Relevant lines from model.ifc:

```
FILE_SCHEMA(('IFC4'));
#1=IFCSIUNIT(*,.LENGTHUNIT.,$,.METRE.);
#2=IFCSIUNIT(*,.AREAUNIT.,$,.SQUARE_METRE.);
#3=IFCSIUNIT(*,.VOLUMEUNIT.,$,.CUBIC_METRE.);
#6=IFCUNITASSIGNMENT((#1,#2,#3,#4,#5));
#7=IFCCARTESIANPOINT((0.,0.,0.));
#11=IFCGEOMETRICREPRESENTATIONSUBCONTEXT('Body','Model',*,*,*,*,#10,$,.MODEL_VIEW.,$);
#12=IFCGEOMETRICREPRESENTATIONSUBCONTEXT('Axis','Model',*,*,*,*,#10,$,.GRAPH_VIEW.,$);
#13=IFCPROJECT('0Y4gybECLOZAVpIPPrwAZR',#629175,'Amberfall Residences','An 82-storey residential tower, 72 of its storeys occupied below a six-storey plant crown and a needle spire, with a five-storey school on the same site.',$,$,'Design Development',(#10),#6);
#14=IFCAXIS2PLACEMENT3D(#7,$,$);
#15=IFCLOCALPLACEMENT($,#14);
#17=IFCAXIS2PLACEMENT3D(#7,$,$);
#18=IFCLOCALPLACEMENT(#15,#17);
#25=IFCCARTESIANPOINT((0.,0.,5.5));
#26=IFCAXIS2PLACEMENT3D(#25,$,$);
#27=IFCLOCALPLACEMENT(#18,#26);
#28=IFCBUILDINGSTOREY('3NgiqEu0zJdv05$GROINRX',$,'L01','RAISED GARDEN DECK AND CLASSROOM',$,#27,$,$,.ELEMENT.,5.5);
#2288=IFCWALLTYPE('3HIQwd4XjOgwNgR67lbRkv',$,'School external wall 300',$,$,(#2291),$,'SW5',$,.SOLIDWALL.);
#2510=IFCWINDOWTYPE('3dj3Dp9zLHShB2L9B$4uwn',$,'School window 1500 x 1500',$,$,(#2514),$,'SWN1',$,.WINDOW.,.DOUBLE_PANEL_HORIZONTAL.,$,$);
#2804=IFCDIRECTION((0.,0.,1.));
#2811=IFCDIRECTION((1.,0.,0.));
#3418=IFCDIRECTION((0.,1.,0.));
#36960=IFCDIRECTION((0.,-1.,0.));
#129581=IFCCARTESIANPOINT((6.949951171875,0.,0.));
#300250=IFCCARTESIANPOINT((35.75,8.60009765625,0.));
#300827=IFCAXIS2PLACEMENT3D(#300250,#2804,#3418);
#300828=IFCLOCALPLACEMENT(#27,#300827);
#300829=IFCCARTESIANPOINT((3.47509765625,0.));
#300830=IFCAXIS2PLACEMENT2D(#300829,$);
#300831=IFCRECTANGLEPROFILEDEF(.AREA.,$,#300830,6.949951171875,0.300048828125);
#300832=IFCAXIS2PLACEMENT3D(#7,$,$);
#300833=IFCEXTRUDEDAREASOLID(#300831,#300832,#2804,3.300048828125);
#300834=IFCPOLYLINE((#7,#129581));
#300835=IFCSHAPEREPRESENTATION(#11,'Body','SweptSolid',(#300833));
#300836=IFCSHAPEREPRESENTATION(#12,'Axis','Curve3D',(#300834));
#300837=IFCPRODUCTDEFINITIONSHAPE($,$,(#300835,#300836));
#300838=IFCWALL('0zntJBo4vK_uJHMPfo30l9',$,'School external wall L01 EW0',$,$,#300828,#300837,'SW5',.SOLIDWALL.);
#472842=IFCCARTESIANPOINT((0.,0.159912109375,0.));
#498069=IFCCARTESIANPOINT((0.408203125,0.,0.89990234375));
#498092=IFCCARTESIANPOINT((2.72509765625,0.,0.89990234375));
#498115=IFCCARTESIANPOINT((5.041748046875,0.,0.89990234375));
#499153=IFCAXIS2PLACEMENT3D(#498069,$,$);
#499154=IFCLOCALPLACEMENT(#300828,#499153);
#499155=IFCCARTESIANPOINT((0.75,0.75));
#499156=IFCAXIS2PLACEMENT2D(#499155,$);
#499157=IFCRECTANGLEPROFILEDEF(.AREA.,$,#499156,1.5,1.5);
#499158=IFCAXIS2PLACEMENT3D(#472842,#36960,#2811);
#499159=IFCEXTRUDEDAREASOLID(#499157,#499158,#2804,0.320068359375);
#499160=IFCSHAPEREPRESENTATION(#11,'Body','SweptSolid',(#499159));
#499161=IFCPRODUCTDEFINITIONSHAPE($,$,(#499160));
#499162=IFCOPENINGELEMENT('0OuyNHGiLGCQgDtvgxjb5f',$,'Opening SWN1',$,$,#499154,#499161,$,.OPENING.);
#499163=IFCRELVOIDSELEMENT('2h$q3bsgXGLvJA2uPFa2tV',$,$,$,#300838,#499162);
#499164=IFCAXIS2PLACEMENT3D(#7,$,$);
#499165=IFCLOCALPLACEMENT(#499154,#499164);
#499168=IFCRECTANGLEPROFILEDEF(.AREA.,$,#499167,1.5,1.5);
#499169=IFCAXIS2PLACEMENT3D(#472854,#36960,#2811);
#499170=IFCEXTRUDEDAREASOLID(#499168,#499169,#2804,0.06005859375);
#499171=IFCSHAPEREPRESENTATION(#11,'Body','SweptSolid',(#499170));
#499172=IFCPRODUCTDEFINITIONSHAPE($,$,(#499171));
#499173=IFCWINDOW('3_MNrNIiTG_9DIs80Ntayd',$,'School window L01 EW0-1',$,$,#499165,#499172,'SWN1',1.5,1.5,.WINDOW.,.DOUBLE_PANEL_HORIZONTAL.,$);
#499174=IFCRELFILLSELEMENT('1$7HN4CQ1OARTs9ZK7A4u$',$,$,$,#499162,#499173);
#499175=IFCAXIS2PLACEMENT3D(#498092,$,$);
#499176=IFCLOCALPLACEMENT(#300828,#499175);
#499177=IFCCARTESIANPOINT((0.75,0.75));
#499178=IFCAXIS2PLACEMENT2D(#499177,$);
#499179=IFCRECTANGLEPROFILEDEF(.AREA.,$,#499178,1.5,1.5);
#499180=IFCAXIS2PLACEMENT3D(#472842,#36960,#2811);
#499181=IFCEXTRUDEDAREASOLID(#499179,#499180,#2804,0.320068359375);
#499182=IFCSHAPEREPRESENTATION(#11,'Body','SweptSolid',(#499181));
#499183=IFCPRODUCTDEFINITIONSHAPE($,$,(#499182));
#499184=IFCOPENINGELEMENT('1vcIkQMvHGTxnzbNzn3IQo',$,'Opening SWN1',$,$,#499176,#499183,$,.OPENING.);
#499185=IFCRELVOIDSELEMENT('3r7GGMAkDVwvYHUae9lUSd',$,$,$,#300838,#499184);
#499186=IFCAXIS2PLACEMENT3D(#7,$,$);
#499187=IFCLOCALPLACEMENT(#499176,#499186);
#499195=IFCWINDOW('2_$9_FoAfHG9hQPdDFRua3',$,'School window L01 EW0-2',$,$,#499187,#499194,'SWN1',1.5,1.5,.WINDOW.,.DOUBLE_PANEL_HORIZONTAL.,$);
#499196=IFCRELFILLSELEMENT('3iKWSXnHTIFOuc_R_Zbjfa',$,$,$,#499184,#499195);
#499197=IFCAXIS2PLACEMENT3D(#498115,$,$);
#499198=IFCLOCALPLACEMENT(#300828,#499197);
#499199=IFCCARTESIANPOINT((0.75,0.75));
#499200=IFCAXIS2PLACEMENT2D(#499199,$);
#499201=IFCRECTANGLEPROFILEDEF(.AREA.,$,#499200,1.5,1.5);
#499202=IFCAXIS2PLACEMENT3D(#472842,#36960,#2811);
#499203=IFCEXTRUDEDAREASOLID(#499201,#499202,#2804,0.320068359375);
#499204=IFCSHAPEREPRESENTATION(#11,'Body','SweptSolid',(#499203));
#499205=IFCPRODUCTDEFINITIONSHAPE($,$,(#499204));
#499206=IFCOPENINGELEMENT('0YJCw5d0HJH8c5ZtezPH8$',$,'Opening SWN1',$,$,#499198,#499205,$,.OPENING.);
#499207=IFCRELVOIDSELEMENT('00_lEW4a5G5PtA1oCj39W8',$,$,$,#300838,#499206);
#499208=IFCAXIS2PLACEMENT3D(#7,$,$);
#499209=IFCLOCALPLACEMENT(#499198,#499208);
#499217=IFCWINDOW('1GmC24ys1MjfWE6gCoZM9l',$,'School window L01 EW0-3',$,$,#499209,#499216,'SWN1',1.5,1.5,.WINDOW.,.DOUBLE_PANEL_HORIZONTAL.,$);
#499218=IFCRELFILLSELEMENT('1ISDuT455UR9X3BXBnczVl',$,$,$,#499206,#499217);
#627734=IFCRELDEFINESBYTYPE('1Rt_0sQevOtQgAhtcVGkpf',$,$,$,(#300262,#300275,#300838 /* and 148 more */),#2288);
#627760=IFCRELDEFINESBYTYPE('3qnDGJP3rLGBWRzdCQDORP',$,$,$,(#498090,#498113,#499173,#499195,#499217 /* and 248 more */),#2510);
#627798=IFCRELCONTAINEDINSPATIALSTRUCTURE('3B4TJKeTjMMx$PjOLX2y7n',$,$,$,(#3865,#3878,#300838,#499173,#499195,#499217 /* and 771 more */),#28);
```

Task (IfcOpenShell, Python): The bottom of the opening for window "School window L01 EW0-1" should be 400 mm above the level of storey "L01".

```python
import numpy as np
import ifcopenshell
import ifcopenshell.api.geometry
import ifcopenshell.geom
import ifcopenshell.util.element
import ifcopenshell.util.placement
import ifcopenshell.util.shape
import ifcopenshell.util.unit

model = ifcopenshell.open("model.ifc")
unit_scale = ifcopenshell.util.unit.calculate_unit_scale(model)

window = model.by_guid("3_MNrNIiTG_9DIs80Ntayd")
opening = window.FillsVoids[0].RelatingOpeningElement
storey = ifcopenshell.util.element.get_container(window, ifc_class="IfcBuildingStorey")
level = ifcopenshell.util.placement.get_local_placement(storey.ObjectPlacement)[2, 3]

# The opening's origin need not be at the sill, so measure its lowest point.
shape = ifcopenshell.geom.create_shape(ifcopenshell.geom.settings(), opening)
bottom = ifcopenshell.util.shape.get_shape_bottom_elevation(shape, shape.geometry) / unit_scale
dz = level + 0.4 / unit_scale - bottom

shift = np.array([0.0, 0.0, dz])
# The window is placed relative to its opening, so it follows when the opening moves.
matrix = ifcopenshell.util.placement.get_local_placement(opening.ObjectPlacement)
matrix[:3, 3] += shift
ifcopenshell.api.geometry.edit_object_placement(
    model, product=opening, matrix=matrix, is_si=False, should_transform_children=True
)

print(f"moved by {dz * unit_scale:+.3f} m")

model.write("model-out.ifc")
```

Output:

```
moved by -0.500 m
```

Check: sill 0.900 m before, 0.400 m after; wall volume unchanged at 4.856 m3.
